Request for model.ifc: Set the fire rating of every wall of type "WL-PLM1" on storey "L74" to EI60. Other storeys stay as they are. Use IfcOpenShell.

First a look at what the model holds.

```python
import ifcopenshell
import ifcopenshell.util.element

model = ifcopenshell.open("model.ifc")
print(model.schema)
storey = next(s for s in model.by_type("IfcBuildingStorey") if s.Name == "L74")
walls = [e for e in ifcopenshell.util.element.get_decomposition(storey) if e.is_a("IfcWall")]
seen = {}
for e in walls:
    element_type = ifcopenshell.util.element.get_type(e)
    key = (element_type.Name if element_type != e and element_type else None, ifcopenshell.util.element.get_pset(e, "Pset_WallCommon", "FireRating"))
    seen[key] = seen.get(key, 0) + 1
for (name, value), count in sorted(seen.items(), key=str):
    print(count, "x", name, "|", value)
```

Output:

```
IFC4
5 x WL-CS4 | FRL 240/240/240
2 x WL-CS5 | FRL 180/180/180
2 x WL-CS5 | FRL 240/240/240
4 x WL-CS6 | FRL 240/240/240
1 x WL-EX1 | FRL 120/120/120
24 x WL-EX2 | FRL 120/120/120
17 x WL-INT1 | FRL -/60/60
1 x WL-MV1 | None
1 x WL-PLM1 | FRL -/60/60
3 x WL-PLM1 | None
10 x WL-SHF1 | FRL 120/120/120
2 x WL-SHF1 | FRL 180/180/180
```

```python
import ifcopenshell
import ifcopenshell.api.pset
import ifcopenshell.util.element

model = ifcopenshell.open("model.ifc")

storey = next(s for s in model.by_type("IfcBuildingStorey") if s.Name == "L74")
walls = [e for e in ifcopenshell.util.element.get_decomposition(storey) if e.is_a("IfcWall")]

count = 0
for e in walls:
    element_type = ifcopenshell.util.element.get_type(e)
    if element_type in (None, e) or element_type.Name != "WL-PLM1":
        continue
    found = ifcopenshell.util.element.get_pset(e, "Pset_WallCommon", should_inherit=False)
    if found:
        pset = model.by_id(found["id"])
        if len(ifcopenshell.util.element.get_elements_by_pset(pset)) > 1:
            pset = ifcopenshell.api.pset.unshare_pset(model, products=[e], pset=pset)[0]
    else:
        pset = ifcopenshell.api.pset.add_pset(model, product=e, name="Pset_WallCommon")
    ifcopenshell.api.pset.edit_pset(model, pset=pset, properties={"FireRating": "EI60"})
    count += 1

print(count, "walls updated")

model.write("model_v2.ifc")
```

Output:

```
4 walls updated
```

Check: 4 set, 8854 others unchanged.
